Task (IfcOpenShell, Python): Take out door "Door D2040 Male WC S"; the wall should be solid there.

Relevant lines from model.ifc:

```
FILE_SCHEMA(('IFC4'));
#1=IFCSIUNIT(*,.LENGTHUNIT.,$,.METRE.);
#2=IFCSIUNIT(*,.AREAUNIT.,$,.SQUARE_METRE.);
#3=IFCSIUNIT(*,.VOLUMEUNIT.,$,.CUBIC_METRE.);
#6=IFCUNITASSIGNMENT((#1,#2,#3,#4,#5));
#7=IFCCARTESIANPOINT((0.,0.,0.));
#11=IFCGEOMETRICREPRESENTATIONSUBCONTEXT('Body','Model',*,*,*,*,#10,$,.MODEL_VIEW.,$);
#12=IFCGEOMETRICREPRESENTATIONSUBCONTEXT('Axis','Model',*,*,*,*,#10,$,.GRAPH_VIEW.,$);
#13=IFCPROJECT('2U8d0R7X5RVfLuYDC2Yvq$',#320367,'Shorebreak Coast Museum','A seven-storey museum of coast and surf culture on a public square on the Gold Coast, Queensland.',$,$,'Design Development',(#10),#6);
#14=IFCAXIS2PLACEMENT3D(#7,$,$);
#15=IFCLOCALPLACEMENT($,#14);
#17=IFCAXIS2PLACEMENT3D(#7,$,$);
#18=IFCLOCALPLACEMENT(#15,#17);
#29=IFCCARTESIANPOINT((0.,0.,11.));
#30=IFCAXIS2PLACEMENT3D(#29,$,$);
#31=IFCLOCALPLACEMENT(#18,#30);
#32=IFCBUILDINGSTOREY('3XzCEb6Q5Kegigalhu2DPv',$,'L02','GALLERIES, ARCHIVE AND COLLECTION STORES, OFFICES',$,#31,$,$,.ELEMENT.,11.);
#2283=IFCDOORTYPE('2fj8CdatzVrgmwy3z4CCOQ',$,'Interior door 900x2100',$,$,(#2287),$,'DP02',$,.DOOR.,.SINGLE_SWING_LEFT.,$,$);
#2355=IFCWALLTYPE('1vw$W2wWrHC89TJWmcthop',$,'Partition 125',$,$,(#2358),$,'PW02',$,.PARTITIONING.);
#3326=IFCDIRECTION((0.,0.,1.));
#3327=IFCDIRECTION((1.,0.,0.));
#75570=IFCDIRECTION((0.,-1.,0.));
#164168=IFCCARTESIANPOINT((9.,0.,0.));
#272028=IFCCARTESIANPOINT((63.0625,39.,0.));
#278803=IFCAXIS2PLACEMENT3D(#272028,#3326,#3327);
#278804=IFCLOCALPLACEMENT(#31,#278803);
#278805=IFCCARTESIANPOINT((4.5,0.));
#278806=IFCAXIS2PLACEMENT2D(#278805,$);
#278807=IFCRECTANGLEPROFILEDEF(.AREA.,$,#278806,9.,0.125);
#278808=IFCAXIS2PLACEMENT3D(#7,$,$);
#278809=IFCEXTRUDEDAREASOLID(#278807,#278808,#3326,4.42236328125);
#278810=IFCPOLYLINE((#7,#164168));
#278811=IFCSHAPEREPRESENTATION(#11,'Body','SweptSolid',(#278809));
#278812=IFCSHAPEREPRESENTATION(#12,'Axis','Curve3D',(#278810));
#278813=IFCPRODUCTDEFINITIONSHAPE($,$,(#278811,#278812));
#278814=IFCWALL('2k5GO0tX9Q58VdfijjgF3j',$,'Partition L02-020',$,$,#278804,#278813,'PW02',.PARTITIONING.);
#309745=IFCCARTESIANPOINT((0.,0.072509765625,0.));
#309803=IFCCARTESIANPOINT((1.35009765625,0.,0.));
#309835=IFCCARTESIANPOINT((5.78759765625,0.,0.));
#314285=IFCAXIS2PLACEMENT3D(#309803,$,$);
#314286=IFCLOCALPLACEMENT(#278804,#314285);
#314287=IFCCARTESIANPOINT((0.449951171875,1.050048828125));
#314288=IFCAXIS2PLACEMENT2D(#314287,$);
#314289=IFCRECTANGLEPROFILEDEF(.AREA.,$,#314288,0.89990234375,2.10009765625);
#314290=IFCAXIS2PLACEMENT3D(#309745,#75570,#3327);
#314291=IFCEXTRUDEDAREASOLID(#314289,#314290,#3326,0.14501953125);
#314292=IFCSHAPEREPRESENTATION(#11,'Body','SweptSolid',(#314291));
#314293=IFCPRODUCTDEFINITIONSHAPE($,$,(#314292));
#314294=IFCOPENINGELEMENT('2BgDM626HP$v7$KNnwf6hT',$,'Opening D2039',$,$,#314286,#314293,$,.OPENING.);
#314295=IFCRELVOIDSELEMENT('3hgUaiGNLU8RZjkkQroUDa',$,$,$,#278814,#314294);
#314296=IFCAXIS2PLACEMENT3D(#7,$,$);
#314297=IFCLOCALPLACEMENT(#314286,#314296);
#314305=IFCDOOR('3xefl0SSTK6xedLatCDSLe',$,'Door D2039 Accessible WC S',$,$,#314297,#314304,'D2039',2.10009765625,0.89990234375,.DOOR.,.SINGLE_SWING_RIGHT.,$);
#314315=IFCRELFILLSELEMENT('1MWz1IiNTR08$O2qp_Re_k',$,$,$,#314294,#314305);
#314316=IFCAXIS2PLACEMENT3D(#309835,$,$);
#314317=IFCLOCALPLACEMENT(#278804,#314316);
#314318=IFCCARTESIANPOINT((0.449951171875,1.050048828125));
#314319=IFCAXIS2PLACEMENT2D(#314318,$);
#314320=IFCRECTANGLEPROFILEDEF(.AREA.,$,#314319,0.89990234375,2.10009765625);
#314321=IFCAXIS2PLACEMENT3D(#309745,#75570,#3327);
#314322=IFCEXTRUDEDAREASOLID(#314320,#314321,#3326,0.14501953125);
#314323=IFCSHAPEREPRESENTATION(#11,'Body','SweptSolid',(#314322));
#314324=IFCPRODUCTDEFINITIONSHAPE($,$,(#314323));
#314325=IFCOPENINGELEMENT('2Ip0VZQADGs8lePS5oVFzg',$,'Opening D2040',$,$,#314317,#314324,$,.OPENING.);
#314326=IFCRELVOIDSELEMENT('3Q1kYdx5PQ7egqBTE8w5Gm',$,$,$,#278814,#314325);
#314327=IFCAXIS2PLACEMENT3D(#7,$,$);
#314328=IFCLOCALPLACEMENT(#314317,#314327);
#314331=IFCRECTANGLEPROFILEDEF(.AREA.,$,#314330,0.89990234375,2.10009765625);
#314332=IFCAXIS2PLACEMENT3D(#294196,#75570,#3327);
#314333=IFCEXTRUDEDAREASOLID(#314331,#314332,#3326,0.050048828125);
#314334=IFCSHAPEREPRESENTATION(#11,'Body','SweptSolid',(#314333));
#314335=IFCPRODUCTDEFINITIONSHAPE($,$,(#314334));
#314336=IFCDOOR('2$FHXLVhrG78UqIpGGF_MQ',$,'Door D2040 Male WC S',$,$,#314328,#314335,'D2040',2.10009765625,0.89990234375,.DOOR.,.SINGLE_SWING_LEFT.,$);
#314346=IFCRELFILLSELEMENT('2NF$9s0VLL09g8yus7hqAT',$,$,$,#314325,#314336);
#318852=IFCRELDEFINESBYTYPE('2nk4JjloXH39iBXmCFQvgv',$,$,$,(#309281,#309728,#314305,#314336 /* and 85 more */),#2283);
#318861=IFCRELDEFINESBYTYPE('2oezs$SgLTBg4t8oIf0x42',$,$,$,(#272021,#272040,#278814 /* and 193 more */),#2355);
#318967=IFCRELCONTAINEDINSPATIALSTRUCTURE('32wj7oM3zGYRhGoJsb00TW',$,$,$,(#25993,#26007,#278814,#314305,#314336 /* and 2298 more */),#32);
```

```python
import ifcopenshell
import ifcopenshell.api.feature
import ifcopenshell.api.root
import ifcopenshell.geom
import ifcopenshell.util.shape

model = ifcopenshell.open("model.ifc")
settings = ifcopenshell.geom.settings()


def volume(element):
    """Net volume in cubic metres, openings subtracted."""
    shape = ifcopenshell.geom.create_shape(settings, element)
    return ifcopenshell.util.shape.get_volume(shape.geometry)


door = model.by_guid("2$FHXLVhrG78UqIpGGF_MQ")
opening = door.FillsVoids[0].RelatingOpeningElement
wall = opening.VoidsElements[0].RelatingBuildingElement
before = volume(wall)

ifcopenshell.api.root.remove_product(model, product=door)
ifcopenshell.api.feature.remove_feature(model, feature=opening)

after = volume(wall)

print(f"wall volume {before:.3f} -> {after:.3f} m3")

model.write("model_rev.ifc")
```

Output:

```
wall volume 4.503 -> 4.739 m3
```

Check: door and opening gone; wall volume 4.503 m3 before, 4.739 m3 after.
